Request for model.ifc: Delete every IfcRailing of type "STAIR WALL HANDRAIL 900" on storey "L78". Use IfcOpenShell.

First a look at what the model holds.

```python
import ifcopenshell
import ifcopenshell.util.element

model = ifcopenshell.open("model.ifc")
print(model.schema)
storey = next(s for s in model.by_type("IfcBuildingStorey") if s.Name == "L78")
railings = [e for e in ifcopenshell.util.element.get_decomposition(storey) if e.is_a("IfcRailing")]
seen = {}
for e in railings:
    element_type = ifcopenshell.util.element.get_type(e)
    name = element_type.Name if element_type not in (None, e) else None
    seen[name] = seen.get(name, 0) + 1
for name, count in sorted(seen.items(), key=str):
    print(count, "x", name)
```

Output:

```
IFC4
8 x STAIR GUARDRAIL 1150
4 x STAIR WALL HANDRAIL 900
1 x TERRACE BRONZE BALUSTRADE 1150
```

```python
import ifcopenshell
import ifcopenshell.api.root
import ifcopenshell.util.element

model = ifcopenshell.open("model.ifc")

storey = next(s for s in model.by_type("IfcBuildingStorey") if s.Name == "L78")
railings = [e for e in ifcopenshell.util.element.get_decomposition(storey) if e.is_a("IfcRailing")]
targets = [e for e in railings if (t := ifcopenshell.util.element.get_type(e)) not in (None, e) and t.Name == "STAIR WALL HANDRAIL 900"]

for e in targets:
    ifcopenshell.api.root.remove_product(model, product=e)
print(len(targets), "removed")

model.write("model_edited.ifc")
```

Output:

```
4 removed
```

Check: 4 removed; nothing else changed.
